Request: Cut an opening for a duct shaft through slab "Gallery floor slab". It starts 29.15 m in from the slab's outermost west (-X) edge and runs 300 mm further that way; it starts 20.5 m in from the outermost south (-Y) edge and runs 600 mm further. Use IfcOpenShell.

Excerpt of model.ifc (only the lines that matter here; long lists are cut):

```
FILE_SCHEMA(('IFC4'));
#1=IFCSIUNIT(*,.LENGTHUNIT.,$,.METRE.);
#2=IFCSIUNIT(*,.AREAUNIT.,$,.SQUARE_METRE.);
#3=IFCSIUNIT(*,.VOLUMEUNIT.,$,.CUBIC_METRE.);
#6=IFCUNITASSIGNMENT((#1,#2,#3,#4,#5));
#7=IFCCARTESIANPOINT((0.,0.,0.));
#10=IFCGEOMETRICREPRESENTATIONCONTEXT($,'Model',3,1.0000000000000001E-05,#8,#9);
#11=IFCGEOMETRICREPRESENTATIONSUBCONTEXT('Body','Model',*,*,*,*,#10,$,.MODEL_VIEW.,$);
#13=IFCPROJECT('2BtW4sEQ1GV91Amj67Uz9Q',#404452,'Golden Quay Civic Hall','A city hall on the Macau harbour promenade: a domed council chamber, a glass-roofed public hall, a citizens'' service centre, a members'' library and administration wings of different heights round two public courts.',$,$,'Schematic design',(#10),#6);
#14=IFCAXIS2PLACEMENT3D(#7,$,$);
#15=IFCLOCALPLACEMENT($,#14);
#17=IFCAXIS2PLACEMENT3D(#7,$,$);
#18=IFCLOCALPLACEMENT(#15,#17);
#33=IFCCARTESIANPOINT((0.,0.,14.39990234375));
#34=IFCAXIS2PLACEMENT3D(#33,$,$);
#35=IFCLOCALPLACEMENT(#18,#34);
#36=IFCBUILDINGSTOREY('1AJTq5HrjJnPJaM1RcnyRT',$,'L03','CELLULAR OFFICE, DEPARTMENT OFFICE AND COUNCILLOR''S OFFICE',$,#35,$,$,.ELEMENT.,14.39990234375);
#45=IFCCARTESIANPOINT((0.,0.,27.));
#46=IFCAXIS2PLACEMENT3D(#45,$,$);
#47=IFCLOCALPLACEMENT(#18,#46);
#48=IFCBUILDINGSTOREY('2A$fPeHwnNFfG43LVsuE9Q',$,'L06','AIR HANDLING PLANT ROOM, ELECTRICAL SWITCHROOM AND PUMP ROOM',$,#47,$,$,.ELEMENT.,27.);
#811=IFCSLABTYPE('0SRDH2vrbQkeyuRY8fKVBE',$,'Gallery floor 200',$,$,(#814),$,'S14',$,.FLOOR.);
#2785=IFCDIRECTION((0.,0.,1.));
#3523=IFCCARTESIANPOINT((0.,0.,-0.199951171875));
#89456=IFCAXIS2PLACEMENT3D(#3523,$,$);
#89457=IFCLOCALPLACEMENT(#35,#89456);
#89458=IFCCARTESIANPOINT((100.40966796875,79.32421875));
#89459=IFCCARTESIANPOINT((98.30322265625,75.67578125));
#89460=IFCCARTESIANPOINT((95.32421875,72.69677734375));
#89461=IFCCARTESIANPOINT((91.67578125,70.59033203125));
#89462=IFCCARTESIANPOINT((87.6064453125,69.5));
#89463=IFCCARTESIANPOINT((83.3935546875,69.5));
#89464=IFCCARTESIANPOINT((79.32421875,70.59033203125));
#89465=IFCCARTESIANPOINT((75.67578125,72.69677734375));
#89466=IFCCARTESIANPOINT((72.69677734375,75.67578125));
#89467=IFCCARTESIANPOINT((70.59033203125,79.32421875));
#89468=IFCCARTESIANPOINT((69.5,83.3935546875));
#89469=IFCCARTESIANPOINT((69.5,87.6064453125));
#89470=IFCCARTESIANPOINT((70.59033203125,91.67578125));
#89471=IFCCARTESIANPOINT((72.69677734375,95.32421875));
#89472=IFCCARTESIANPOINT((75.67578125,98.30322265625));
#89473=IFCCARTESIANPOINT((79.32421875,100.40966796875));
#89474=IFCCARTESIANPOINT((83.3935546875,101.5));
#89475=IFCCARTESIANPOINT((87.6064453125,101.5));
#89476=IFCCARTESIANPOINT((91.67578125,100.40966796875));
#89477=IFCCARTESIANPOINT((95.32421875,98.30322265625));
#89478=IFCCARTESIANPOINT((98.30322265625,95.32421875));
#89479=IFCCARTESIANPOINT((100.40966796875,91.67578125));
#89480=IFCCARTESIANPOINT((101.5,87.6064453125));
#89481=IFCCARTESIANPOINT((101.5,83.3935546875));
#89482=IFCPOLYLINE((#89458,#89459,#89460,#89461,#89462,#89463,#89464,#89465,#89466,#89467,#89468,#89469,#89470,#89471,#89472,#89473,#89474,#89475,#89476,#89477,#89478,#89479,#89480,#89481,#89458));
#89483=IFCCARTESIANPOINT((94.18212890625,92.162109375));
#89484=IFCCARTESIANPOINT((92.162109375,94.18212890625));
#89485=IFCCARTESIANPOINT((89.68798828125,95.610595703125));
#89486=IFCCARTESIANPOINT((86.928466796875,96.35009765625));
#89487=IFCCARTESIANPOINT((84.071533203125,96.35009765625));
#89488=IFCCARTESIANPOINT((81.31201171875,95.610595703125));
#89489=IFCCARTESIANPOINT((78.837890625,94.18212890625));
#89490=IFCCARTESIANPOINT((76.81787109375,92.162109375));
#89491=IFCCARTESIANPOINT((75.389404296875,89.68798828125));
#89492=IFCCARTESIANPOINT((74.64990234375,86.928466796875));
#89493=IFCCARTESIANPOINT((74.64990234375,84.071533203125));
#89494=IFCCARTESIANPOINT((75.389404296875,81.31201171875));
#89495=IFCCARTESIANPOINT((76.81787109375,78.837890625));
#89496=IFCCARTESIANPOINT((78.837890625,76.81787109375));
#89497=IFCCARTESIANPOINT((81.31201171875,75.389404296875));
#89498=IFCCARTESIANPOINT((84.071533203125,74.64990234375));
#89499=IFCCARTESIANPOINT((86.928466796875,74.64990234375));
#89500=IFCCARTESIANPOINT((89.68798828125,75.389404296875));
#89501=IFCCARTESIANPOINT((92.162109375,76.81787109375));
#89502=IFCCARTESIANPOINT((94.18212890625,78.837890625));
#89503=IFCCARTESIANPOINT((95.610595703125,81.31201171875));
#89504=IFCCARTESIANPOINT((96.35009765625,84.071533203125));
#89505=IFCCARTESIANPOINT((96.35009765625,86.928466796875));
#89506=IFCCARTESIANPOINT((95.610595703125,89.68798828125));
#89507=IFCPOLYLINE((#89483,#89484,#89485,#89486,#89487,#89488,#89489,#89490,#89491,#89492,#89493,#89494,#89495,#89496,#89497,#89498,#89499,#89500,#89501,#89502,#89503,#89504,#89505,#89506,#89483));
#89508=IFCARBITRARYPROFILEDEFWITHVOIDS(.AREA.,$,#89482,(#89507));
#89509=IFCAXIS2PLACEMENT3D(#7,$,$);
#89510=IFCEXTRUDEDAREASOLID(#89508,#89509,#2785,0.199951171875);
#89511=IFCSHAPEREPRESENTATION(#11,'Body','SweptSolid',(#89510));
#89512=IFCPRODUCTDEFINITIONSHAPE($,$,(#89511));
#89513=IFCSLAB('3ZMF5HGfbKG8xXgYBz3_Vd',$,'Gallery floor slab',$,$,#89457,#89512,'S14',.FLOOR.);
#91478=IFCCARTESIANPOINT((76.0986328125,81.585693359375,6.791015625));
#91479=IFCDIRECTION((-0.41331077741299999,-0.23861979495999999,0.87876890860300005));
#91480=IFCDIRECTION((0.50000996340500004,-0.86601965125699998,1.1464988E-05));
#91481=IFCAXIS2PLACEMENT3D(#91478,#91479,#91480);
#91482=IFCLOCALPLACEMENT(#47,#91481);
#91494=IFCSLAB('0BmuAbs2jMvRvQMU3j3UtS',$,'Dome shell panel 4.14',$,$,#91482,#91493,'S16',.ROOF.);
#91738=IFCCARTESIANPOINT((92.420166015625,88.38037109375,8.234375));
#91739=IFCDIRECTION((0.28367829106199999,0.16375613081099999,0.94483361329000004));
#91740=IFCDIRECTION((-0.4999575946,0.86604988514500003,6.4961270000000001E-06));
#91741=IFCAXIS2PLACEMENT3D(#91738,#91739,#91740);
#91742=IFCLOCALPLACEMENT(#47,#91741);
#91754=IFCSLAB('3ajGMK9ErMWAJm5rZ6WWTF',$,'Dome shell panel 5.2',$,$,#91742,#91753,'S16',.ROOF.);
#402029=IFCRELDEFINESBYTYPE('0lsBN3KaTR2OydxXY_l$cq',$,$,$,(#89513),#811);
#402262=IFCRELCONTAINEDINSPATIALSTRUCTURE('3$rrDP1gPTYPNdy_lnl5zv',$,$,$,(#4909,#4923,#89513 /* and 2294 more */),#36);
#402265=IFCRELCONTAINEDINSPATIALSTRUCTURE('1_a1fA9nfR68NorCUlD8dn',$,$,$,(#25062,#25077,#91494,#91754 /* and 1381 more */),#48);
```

```python
import numpy as np
import ifcopenshell
import ifcopenshell.api.feature
import ifcopenshell.api.geometry
import ifcopenshell.api.root
import ifcopenshell.geom
import ifcopenshell.util.placement
import ifcopenshell.util.representation
import ifcopenshell.util.shape
import ifcopenshell.util.unit

model = ifcopenshell.open("model.ifc")
unit_scale = ifcopenshell.util.unit.calculate_unit_scale(model)
settings = ifcopenshell.geom.settings()


def volume(element):
    """Net volume in cubic metres, openings subtracted."""
    shape = ifcopenshell.geom.create_shape(settings, element)
    return ifcopenshell.util.shape.get_volume(shape.geometry)


slab = model.by_guid("3ZMF5HGfbKG8xXgYBz3_Vd")
before = volume(slab)

# Extent in the slab's own axes, in metres. The edges named are its -X and -Y sides.
slab_shape = ifcopenshell.geom.create_shape(settings, slab)
vertices = ifcopenshell.util.shape.get_vertices(slab_shape.geometry)
x_min, y_min, bottom = vertices.min(axis=0)
top = vertices[:, 2].max()

opening = ifcopenshell.api.root.create_entity(model, ifc_class="IfcOpeningElement", name="Duct shaft opening", predefined_type="OPENING")
context = ifcopenshell.util.representation.get_context(model, "Model", "Body", "MODEL_VIEW")
width, depth = 0.3, 0.6
outline = [(0.0, 0.0), (width, 0.0), (width, depth), (0.0, depth), (0.0, 0.0)]
# Overshoot both faces by 50 mm so the cut is clean.
shape = ifcopenshell.api.geometry.add_slab_representation(
    model, context=context, depth=top - bottom + 0.1, polyline=outline
)
ifcopenshell.api.geometry.assign_representation(model, product=opening, representation=shape)

matrix = ifcopenshell.util.placement.get_local_placement(slab.ObjectPlacement)
matrix[:, 3] = matrix @ np.append(np.array([x_min + 29.15, y_min + 20.5, bottom - 0.05]) / unit_scale, 1.0)
ifcopenshell.api.geometry.edit_object_placement(model, product=opening, matrix=matrix, is_si=False)
ifcopenshell.api.feature.add_feature(model, feature=opening, element=slab)

after = volume(slab)

print(f"slab volume {before:.3f} -> {after:.3f} m3")

model.write("model-out.ifc")
```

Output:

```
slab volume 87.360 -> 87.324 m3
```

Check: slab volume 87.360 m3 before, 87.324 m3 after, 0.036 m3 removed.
